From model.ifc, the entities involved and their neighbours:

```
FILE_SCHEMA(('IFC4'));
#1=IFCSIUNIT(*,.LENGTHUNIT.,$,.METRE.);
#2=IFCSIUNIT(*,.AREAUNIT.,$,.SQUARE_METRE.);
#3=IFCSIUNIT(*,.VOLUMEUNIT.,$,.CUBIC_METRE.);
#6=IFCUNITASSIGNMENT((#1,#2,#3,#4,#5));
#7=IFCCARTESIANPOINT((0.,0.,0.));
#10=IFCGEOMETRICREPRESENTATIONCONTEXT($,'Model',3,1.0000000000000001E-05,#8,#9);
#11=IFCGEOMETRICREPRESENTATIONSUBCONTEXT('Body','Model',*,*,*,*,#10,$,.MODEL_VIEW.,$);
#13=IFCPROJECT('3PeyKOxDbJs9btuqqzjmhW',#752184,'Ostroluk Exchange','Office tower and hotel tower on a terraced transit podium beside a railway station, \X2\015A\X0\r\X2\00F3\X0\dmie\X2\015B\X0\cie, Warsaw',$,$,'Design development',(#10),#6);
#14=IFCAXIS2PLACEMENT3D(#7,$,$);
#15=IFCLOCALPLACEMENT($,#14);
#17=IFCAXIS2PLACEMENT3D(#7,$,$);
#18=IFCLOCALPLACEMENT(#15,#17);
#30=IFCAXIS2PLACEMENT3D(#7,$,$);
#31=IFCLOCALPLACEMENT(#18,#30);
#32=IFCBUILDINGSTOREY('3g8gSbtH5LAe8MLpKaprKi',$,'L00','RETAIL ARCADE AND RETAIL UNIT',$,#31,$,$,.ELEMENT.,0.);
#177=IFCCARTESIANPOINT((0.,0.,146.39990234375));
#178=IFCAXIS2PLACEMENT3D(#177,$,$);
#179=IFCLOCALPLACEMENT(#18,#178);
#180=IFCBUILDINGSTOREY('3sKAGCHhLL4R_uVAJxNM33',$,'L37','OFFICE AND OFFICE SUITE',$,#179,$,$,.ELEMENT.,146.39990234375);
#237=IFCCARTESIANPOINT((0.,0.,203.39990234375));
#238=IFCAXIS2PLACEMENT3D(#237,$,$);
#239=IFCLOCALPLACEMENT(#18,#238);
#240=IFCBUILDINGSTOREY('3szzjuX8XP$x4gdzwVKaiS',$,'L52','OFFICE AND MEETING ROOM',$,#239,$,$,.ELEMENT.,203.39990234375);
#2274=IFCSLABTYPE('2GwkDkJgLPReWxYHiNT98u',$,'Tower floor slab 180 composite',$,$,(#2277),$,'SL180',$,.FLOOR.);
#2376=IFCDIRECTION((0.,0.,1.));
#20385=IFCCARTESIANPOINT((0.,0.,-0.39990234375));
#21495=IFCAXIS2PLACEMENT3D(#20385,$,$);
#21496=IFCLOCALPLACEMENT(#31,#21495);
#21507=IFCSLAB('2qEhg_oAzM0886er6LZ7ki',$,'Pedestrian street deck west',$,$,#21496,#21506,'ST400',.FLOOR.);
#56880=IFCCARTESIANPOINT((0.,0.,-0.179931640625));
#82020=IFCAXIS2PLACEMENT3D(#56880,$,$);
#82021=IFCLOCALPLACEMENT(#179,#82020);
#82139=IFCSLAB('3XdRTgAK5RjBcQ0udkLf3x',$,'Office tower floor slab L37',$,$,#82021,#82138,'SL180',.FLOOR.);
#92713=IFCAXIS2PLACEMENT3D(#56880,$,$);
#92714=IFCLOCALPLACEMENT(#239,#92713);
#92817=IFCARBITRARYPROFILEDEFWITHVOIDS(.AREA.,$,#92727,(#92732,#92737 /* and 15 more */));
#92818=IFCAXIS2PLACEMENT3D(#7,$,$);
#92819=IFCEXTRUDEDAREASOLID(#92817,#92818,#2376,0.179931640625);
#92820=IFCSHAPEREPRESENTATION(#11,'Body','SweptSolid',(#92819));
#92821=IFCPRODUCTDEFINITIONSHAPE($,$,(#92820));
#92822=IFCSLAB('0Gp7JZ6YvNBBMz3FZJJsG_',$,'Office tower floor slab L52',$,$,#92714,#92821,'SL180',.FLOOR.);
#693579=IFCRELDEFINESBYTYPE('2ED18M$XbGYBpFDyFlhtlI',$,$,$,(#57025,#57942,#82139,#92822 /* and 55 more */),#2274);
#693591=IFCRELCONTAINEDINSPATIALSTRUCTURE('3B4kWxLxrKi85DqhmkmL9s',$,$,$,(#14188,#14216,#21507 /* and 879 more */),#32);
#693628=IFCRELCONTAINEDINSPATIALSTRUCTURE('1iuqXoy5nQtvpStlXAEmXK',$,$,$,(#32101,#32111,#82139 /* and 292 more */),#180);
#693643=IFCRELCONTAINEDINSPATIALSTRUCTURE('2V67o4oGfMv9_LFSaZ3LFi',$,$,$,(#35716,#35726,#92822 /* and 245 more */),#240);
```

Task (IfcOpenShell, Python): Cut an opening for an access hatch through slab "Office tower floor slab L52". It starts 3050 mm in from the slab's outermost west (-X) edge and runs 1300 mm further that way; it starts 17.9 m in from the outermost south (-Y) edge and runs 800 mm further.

```python
import numpy as np
import ifcopenshell
import ifcopenshell.api.feature
import ifcopenshell.api.geometry
import ifcopenshell.api.root
import ifcopenshell.geom
import ifcopenshell.util.placement
import ifcopenshell.util.representation
import ifcopenshell.util.shape
import ifcopenshell.util.unit

model = ifcopenshell.open("model.ifc")
unit_scale = ifcopenshell.util.unit.calculate_unit_scale(model)
settings = ifcopenshell.geom.settings()


def volume(element):
    """Net volume in cubic metres, openings subtracted."""
    shape = ifcopenshell.geom.create_shape(settings, element)
    return ifcopenshell.util.shape.get_volume(shape.geometry)


slab = model.by_guid("0Gp7JZ6YvNBBMz3FZJJsG_")
before = volume(slab)

# Extent in the slab's own axes, in metres. The edges named are its -X and -Y sides.
slab_shape = ifcopenshell.geom.create_shape(settings, slab)
vertices = ifcopenshell.util.shape.get_vertices(slab_shape.geometry)
x_min, y_min, bottom = vertices.min(axis=0)
top = vertices[:, 2].max()

opening = ifcopenshell.api.root.create_entity(model, ifc_class="IfcOpeningElement", name="Access hatch opening", predefined_type="OPENING")
context = ifcopenshell.util.representation.get_context(model, "Model", "Body", "MODEL_VIEW")
width, depth = 1.3, 0.8
outline = [(0.0, 0.0), (width, 0.0), (width, depth), (0.0, depth), (0.0, 0.0)]
# Overshoot both faces by 50 mm so the cut is clean.
shape = ifcopenshell.api.geometry.add_slab_representation(
    model, context=context, depth=top - bottom + 0.1, polyline=outline
)
ifcopenshell.api.geometry.assign_representation(model, product=opening, representation=shape)

matrix = ifcopenshell.util.placement.get_local_placement(slab.ObjectPlacement)
matrix[:, 3] = matrix @ np.append(np.array([x_min + 3.05, y_min + 17.9, bottom - 0.05]) / unit_scale, 1.0)
ifcopenshell.api.geometry.edit_object_placement(model, product=opening, matrix=matrix, is_si=False)
ifcopenshell.api.feature.add_feature(model, feature=opening, element=slab)

after = volume(slab)

print(f"slab volume {before:.3f} -> {after:.3f} m3")

model.write("model_edited.ifc")
```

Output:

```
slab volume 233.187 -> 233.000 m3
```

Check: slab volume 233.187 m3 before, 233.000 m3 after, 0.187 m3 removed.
